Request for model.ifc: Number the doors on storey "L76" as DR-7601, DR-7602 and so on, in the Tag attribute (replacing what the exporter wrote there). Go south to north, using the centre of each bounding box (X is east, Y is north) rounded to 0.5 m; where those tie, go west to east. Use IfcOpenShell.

First a look at what the model holds.

```python
import ifcopenshell
import ifcopenshell.util.element
import ifcopenshell.util.placement

model = ifcopenshell.open("model.ifc")
print(model.schema)
storey = next(s for s in model.by_type("IfcBuildingStorey") if s.Name == "L76")
doors = [e for e in ifcopenshell.util.element.get_decomposition(storey) if e.is_a("IfcDoor")]
for e in sorted(doors, key=lambda e: e.id()):
    origin = ifcopenshell.util.placement.get_local_placement(e.ObjectPlacement)[:3, 3]
    print(e.id(), e.Tag, e.Name, origin.round(2) + 0.0, sep=" | ")
```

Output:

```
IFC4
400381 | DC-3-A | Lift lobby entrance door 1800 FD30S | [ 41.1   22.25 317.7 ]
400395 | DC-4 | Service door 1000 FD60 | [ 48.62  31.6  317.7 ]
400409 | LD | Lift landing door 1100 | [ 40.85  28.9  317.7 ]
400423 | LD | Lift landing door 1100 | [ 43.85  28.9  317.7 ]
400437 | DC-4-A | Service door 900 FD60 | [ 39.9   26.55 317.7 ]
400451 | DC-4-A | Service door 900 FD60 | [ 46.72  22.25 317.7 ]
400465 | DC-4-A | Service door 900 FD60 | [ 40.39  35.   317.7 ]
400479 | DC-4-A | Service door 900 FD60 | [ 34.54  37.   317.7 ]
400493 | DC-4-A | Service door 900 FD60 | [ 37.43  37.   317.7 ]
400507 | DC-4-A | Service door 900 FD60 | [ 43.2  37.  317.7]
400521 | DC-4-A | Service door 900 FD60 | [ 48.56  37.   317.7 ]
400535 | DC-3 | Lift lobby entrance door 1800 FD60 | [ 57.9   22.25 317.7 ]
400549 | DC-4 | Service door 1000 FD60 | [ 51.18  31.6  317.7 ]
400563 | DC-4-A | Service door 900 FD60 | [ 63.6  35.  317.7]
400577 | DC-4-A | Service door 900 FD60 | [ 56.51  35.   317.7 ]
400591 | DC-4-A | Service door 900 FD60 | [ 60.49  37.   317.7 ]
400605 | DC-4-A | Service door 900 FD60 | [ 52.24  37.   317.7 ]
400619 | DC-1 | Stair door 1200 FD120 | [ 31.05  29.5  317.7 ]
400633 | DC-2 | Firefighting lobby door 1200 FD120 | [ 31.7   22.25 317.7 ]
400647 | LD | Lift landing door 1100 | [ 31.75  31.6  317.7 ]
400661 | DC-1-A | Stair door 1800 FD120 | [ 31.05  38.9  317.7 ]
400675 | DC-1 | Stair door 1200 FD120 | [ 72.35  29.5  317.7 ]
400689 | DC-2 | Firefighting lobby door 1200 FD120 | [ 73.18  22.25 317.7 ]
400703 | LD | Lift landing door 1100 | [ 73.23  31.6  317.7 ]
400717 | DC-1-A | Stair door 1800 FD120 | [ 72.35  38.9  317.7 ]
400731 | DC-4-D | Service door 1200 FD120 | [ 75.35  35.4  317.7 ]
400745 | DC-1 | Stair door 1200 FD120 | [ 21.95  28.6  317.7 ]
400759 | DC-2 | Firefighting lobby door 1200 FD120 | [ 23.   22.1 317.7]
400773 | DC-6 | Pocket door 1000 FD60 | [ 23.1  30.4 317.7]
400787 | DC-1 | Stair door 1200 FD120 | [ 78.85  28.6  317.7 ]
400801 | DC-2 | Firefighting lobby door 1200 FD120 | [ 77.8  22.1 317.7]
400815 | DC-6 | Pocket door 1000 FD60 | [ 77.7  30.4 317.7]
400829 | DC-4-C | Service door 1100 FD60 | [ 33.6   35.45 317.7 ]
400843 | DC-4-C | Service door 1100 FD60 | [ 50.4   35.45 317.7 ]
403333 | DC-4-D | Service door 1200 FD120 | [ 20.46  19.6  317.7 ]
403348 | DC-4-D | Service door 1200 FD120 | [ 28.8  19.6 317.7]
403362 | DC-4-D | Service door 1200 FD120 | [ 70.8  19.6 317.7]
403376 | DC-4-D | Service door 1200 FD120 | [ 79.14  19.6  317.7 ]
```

```python
import ifcopenshell
import ifcopenshell.geom
import ifcopenshell.util.element
import ifcopenshell.util.shape

model = ifcopenshell.open("model.ifc")
settings = ifcopenshell.geom.settings()
settings.set("use-world-coords", True)


def centre(element):
    shape = ifcopenshell.geom.create_shape(settings, element)
    return ifcopenshell.util.shape.get_bbox_centroid(shape.geometry)


storey = next(s for s in model.by_type("IfcBuildingStorey") if s.Name == "L76")
doors = [e for e in ifcopenshell.util.element.get_decomposition(storey) if e.is_a("IfcDoor")]

# Insertion points can sit at a corner or the storey origin, so sort by the geometry (in metres).
centres = {e: centre(e) for e in doors}
doors.sort(key=lambda e: (round(centres[e][1] / 0.5), centres[e][0]))

for i, e in enumerate(doors, start=1):
    number = f"DR-76{i:02d}"
    e.Tag = number
    print(e.id(), number)

model.write("model-out.ifc")
```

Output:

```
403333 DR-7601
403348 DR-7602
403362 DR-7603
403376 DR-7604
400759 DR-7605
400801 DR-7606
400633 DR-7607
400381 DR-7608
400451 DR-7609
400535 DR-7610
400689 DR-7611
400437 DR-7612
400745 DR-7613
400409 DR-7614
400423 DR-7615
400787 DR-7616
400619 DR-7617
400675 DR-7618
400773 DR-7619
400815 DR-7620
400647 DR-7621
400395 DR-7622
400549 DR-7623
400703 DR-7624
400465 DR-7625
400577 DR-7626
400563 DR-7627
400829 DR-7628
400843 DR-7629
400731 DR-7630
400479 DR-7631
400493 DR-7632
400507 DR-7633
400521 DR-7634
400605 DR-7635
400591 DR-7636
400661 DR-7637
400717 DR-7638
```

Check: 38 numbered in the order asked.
